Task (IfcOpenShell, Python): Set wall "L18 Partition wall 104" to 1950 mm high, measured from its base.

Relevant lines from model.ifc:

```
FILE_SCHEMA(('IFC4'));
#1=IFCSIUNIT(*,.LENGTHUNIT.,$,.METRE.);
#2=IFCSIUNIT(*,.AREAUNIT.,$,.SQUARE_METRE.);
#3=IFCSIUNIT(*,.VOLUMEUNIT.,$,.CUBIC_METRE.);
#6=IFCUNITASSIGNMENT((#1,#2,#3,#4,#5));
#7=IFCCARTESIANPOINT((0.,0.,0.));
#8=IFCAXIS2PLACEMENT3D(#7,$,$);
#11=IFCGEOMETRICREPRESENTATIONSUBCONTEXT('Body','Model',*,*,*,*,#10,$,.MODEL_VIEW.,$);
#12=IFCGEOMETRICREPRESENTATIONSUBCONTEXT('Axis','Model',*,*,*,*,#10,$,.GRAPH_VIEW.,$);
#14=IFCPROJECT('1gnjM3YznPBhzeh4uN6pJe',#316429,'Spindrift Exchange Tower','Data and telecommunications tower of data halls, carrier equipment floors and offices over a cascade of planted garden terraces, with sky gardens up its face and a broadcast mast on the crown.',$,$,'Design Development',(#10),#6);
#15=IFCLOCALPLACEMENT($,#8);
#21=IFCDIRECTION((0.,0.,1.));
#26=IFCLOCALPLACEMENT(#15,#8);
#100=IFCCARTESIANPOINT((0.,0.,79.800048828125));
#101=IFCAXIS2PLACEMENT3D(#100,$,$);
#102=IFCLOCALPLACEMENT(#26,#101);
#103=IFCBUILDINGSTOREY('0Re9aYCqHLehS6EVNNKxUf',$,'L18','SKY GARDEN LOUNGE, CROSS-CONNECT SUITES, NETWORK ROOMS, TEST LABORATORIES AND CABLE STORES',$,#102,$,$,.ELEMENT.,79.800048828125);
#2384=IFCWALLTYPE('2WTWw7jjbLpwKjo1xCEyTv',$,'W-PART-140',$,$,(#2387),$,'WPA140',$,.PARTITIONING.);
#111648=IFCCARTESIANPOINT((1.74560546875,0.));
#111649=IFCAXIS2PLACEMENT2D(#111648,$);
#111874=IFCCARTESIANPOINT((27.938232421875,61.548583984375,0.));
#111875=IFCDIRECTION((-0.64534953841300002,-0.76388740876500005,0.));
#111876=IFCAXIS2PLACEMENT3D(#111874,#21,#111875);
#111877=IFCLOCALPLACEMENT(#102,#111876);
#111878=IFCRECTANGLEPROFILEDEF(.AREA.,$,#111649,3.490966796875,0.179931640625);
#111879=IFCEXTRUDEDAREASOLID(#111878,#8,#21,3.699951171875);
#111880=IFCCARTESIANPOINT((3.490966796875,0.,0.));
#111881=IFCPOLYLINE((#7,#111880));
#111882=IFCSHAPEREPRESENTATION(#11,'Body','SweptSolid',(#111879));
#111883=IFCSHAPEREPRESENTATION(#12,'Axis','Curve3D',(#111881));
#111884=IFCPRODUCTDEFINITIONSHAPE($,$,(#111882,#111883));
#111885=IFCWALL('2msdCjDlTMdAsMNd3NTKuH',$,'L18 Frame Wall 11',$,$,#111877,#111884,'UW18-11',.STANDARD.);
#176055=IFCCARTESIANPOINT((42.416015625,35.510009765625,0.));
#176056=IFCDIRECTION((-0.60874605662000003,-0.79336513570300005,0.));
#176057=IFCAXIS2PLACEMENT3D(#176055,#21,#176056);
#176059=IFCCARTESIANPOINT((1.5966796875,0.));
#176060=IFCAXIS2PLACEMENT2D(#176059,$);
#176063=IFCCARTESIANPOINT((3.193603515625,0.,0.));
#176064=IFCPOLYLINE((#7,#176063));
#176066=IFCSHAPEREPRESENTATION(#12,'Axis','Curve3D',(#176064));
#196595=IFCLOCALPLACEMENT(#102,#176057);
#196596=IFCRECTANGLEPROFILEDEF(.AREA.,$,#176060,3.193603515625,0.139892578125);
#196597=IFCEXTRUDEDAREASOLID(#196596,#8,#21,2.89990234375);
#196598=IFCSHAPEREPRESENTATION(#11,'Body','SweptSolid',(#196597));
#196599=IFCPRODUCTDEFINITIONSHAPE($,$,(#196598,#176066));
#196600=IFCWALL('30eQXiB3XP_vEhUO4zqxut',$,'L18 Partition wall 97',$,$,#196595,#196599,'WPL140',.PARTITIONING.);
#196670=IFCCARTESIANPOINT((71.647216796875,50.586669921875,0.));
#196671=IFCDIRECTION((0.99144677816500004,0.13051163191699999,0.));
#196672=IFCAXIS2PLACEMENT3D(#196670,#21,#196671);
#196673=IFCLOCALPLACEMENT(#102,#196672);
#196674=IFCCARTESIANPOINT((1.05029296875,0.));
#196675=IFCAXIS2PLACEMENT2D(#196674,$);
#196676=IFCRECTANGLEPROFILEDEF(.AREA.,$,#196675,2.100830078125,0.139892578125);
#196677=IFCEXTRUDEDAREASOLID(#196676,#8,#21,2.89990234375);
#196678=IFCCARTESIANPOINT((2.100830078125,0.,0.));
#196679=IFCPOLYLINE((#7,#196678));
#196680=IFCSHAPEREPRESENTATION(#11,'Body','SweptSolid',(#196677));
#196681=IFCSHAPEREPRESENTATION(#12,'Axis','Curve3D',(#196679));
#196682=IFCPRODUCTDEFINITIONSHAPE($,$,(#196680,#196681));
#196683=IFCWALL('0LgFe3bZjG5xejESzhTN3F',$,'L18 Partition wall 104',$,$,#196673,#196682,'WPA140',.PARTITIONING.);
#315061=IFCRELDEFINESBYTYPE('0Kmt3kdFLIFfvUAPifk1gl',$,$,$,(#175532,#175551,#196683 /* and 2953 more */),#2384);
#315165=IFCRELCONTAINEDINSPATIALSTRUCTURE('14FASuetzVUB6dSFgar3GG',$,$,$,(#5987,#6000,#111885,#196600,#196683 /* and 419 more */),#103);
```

```python
import ifcopenshell
import ifcopenshell.geom
import ifcopenshell.util.representation
import ifcopenshell.util.shape
import ifcopenshell.util.unit

model = ifcopenshell.open("model.ifc")
unit_scale = ifcopenshell.util.unit.calculate_unit_scale(model)
settings = ifcopenshell.geom.settings()


def volume(element):
    """Net volume in cubic metres, openings subtracted."""
    shape = ifcopenshell.geom.create_shape(settings, element)
    return ifcopenshell.util.shape.get_volume(shape.geometry)


wall = model.by_guid("0LgFe3bZjG5xejESzhTN3F")
before = volume(wall)

body = ifcopenshell.util.representation.get_representation(wall, "Model", "Body")
solid = body.Items[0]
old_height = solid.Depth
solid.Depth = 1.95 / unit_scale
after = volume(wall)

print(f"height {old_height:g} -> {solid.Depth:g}, volume {before:.3f} -> {after:.3f} m3")

model.write("model_rev.ifc")
```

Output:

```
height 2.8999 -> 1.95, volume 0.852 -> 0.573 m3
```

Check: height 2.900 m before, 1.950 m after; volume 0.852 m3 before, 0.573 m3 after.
